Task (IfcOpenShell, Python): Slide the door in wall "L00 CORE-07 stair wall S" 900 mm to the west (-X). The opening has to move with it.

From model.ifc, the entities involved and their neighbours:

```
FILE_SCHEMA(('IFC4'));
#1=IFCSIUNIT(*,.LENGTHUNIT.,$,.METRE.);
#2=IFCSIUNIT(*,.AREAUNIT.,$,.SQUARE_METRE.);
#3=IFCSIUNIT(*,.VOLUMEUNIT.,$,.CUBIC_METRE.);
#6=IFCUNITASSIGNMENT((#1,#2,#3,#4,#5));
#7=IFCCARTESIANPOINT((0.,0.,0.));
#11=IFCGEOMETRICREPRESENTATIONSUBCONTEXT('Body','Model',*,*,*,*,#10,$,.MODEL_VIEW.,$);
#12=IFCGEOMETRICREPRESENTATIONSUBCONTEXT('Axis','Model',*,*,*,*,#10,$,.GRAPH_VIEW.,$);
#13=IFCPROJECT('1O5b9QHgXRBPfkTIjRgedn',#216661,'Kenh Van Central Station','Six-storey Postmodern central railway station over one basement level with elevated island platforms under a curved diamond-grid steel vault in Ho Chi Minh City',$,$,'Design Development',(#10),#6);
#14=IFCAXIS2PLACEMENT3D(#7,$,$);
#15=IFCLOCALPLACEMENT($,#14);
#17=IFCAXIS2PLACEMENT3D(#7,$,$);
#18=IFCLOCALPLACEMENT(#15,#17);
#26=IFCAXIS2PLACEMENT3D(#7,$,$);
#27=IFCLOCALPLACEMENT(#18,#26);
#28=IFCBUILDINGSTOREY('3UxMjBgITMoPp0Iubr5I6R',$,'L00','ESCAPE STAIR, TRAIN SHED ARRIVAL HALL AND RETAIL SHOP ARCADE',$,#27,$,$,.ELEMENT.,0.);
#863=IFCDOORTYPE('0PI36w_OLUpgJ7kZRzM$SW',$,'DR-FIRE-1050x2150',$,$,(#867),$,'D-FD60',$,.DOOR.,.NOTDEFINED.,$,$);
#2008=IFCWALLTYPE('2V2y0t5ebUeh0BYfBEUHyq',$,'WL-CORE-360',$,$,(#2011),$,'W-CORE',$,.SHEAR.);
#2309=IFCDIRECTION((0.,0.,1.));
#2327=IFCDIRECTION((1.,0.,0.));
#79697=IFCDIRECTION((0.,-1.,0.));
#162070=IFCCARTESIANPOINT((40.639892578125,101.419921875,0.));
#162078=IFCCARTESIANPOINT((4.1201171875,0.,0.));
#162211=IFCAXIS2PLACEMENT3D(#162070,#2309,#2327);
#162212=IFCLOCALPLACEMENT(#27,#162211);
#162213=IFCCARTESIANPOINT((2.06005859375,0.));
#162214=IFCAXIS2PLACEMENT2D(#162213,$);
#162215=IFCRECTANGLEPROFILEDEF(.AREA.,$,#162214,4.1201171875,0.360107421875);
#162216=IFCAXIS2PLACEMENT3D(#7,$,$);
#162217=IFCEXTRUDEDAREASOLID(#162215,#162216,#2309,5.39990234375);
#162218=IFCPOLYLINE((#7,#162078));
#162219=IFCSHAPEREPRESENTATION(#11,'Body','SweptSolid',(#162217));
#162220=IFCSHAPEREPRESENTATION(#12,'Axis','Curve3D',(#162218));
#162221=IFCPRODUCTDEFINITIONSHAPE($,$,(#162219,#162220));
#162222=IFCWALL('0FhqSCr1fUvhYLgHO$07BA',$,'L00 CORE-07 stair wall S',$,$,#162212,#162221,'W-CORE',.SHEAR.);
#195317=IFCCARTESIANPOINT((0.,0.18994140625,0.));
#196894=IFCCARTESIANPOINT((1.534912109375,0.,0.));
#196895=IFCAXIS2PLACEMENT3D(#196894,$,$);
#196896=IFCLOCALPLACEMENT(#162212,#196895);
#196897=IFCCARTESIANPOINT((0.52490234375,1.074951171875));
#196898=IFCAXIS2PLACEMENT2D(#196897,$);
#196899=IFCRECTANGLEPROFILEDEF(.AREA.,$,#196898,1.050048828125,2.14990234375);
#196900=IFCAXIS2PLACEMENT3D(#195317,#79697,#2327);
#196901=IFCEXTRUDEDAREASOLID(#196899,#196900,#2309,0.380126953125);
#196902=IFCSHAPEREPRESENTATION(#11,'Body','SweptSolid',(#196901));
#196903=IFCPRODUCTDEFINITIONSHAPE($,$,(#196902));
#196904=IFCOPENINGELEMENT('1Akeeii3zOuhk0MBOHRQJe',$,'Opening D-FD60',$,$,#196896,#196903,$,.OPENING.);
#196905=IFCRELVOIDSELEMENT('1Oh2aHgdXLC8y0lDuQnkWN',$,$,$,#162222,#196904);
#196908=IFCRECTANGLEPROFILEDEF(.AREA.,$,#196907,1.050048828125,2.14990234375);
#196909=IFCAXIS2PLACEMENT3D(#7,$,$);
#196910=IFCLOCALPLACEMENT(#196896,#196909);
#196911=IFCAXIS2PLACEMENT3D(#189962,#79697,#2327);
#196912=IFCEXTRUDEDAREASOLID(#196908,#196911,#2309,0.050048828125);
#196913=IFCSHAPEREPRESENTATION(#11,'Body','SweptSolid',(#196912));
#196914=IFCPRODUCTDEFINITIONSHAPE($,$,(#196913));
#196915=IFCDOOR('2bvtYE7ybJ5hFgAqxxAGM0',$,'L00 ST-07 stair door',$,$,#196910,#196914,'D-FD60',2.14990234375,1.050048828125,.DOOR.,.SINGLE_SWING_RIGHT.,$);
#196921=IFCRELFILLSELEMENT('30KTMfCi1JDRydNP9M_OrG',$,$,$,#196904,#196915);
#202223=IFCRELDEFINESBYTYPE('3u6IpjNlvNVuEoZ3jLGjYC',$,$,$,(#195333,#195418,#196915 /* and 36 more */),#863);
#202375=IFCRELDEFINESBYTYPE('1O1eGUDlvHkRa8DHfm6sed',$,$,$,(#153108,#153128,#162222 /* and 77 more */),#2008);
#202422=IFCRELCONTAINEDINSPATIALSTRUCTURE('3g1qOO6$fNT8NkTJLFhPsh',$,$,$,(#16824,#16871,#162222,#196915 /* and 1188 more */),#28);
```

```python
import ifcopenshell
import ifcopenshell.api.geometry
import ifcopenshell.util.placement

model = ifcopenshell.open("model.ifc")

door = model.by_guid("2bvtYE7ybJ5hFgAqxxAGM0")
opening = door.FillsVoids[0].RelatingOpeningElement
wall = opening.VoidsElements[0].RelatingBuildingElement

wall_matrix = ifcopenshell.util.placement.get_local_placement(wall.ObjectPlacement)
shift = wall_matrix[:3, 0] * -0.9
before = ifcopenshell.util.placement.get_local_placement(door.ObjectPlacement)[:3, 3].copy()

# The door is placed relative to its opening, so it follows when the opening moves.
matrix = ifcopenshell.util.placement.get_local_placement(opening.ObjectPlacement)
matrix[:3, 3] += shift
ifcopenshell.api.geometry.edit_object_placement(
    model, product=opening, matrix=matrix, is_si=False, should_transform_children=True
)

after = ifcopenshell.util.placement.get_local_placement(door.ObjectPlacement)[:3, 3]
print("door moved by", (after - before).round(3) + 0.0)

model.write("model_v2.ifc")
```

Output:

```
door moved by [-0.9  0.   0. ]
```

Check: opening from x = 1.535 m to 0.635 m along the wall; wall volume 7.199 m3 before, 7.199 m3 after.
